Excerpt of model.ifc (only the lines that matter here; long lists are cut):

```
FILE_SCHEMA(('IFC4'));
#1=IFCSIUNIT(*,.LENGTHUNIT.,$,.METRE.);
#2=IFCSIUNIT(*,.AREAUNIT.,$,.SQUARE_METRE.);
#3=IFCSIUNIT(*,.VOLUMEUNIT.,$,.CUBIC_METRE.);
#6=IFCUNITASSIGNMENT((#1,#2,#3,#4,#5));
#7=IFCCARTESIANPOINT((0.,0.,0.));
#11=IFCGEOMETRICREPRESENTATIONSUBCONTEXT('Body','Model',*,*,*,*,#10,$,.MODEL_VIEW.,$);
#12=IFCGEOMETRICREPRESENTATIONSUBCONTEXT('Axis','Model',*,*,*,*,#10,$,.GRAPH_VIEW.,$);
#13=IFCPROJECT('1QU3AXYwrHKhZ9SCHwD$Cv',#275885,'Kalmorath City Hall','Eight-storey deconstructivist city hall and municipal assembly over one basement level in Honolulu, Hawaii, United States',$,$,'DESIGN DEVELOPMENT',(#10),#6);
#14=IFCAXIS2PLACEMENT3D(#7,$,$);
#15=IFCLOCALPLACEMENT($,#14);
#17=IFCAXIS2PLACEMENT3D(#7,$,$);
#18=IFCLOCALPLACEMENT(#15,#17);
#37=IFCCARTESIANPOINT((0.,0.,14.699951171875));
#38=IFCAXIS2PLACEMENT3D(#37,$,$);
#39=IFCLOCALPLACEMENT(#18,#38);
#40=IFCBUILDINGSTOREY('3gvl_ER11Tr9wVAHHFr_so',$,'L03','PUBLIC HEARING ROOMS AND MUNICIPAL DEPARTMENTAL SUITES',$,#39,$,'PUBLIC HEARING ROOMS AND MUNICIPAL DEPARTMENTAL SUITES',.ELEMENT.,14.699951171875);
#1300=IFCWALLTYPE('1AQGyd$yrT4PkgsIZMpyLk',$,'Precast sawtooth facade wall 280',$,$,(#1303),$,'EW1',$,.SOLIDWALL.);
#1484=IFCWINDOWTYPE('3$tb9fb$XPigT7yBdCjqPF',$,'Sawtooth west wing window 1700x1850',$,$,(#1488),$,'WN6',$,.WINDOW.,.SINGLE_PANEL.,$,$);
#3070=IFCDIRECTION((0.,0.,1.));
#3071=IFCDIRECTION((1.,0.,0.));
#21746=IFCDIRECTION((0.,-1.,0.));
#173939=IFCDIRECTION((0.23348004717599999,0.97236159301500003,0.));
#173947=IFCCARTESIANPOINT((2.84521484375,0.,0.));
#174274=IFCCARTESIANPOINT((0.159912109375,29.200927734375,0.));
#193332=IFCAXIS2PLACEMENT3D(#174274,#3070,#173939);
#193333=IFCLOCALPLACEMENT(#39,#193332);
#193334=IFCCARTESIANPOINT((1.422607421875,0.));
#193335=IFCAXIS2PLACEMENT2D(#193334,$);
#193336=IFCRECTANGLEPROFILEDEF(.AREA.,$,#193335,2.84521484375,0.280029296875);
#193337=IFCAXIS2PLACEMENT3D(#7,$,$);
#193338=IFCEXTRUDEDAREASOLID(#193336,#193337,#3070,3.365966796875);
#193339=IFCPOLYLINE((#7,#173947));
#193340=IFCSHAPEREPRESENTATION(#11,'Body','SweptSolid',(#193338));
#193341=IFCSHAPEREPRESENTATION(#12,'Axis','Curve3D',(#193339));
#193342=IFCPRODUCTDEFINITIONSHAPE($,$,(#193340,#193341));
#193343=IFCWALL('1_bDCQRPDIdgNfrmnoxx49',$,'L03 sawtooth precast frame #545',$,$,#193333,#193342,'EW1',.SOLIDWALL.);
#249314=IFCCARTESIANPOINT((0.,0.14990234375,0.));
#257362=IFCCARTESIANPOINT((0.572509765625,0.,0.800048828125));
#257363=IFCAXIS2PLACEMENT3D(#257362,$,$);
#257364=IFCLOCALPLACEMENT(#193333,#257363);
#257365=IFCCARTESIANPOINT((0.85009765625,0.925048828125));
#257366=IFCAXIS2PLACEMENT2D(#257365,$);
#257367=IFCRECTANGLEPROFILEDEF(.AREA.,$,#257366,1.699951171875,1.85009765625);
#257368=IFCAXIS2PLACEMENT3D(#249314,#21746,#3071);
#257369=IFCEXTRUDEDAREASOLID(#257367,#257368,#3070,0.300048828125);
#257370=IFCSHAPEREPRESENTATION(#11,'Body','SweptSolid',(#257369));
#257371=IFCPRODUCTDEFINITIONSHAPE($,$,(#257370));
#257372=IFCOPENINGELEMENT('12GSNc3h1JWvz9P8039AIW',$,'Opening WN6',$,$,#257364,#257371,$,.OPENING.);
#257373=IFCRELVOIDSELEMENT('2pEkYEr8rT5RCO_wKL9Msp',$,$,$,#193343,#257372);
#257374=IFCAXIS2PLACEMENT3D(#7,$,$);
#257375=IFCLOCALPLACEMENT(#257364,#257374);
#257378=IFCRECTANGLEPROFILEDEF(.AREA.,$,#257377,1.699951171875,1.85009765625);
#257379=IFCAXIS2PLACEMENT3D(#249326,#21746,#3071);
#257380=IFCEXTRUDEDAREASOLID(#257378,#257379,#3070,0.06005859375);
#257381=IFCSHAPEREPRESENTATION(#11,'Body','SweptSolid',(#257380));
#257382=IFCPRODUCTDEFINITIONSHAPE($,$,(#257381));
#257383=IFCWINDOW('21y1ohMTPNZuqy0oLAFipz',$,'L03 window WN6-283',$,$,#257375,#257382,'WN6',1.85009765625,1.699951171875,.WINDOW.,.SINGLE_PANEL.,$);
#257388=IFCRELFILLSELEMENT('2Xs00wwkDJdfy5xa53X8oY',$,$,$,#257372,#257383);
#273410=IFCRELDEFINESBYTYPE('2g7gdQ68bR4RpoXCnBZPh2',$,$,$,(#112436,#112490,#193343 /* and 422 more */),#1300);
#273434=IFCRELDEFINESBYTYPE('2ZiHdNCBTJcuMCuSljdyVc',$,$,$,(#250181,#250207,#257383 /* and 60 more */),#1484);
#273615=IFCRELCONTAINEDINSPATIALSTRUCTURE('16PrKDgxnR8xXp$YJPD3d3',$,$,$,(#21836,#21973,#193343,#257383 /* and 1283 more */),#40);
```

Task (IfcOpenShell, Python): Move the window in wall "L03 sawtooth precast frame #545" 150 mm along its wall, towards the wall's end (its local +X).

```python
import ifcopenshell
import ifcopenshell.api.geometry
import ifcopenshell.util.placement

model = ifcopenshell.open("model.ifc")

window = model.by_guid("21y1ohMTPNZuqy0oLAFipz")
opening = window.FillsVoids[0].RelatingOpeningElement
wall = opening.VoidsElements[0].RelatingBuildingElement

wall_matrix = ifcopenshell.util.placement.get_local_placement(wall.ObjectPlacement)
shift = wall_matrix[:3, 0] * 0.15
before = ifcopenshell.util.placement.get_local_placement(window.ObjectPlacement)[:3, 3].copy()

# The window is placed relative to its opening, so it follows when the opening moves.
matrix = ifcopenshell.util.placement.get_local_placement(opening.ObjectPlacement)
matrix[:3, 3] += shift
ifcopenshell.api.geometry.edit_object_placement(
    model, product=opening, matrix=matrix, is_si=False, should_transform_children=True
)

after = ifcopenshell.util.placement.get_local_placement(window.ObjectPlacement)[:3, 3]
print("window moved by", (after - before).round(3) + 0.0)

model.write("model_v2.ifc")
```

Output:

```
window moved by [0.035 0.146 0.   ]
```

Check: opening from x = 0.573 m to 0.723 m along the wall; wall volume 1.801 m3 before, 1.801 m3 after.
